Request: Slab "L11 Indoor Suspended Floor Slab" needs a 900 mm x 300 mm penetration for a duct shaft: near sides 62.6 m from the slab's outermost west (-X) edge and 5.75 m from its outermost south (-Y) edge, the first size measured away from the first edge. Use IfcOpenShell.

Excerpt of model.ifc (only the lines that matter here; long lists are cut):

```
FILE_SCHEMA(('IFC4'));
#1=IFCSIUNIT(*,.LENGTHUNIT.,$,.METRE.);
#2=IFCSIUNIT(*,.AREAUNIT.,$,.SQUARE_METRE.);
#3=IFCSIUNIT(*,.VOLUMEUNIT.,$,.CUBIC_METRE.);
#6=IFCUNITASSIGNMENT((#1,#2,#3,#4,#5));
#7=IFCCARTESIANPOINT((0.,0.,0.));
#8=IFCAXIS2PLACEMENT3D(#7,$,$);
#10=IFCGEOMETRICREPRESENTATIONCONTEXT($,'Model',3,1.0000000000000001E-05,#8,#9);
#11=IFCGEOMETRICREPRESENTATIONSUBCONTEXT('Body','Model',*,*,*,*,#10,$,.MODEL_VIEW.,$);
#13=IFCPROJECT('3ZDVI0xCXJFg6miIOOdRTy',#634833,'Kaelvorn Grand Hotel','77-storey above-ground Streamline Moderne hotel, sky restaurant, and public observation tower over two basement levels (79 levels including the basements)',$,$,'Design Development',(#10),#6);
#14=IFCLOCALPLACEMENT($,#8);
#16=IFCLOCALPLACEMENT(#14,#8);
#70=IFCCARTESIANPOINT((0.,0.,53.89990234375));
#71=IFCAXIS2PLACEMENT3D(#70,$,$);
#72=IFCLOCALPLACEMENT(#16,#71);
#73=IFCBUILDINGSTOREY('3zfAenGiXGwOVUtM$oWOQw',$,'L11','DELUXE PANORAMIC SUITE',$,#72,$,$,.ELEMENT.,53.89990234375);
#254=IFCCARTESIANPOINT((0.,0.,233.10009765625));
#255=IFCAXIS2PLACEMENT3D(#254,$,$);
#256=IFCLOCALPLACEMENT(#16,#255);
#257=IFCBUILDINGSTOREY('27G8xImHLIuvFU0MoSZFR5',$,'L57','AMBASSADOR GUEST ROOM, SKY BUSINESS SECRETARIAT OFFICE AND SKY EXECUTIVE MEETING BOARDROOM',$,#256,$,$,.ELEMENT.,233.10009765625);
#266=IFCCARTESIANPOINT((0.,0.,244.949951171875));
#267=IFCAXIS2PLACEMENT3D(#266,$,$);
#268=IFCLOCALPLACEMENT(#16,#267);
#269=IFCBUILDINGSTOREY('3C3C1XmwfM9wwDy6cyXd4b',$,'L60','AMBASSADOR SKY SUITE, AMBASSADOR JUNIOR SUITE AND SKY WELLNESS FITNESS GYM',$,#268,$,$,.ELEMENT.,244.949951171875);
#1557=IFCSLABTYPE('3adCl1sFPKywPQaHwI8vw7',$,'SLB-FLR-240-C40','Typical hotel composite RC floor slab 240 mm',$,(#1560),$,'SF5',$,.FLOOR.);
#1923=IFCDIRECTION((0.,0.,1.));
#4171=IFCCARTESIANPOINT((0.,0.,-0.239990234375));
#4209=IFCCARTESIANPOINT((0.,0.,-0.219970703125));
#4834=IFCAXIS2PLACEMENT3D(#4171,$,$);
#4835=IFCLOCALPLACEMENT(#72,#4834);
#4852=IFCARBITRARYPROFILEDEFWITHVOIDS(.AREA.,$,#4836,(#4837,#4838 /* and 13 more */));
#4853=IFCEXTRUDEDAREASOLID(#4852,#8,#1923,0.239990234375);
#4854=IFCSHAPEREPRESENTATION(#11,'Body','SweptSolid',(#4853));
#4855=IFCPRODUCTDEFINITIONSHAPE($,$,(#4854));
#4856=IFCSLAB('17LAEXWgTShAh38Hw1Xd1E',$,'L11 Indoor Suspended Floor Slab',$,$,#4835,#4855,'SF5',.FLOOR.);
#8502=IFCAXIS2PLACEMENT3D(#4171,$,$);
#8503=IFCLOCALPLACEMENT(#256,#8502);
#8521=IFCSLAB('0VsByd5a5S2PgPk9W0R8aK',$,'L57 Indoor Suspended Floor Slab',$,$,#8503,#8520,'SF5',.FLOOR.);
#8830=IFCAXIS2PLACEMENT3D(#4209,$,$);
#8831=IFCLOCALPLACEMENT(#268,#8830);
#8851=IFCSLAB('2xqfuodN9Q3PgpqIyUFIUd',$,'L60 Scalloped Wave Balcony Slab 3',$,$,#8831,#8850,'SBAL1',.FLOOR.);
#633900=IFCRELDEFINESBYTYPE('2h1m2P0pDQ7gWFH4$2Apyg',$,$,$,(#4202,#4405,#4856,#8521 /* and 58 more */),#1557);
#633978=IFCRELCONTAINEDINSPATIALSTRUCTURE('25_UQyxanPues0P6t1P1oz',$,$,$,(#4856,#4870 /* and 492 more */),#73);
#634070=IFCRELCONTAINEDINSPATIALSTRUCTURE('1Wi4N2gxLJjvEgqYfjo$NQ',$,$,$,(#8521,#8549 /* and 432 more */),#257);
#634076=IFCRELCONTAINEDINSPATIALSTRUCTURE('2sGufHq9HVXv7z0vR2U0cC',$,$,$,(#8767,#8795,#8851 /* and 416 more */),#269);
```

```python
import numpy as np
import ifcopenshell
import ifcopenshell.api.feature
import ifcopenshell.api.geometry
import ifcopenshell.api.root
import ifcopenshell.geom
import ifcopenshell.util.placement
import ifcopenshell.util.representation
import ifcopenshell.util.shape
import ifcopenshell.util.unit

model = ifcopenshell.open("model.ifc")
unit_scale = ifcopenshell.util.unit.calculate_unit_scale(model)
settings = ifcopenshell.geom.settings()


def volume(element):
    """Net volume in cubic metres, openings subtracted."""
    shape = ifcopenshell.geom.create_shape(settings, element)
    return ifcopenshell.util.shape.get_volume(shape.geometry)


slab = model.by_guid("17LAEXWgTShAh38Hw1Xd1E")
before = volume(slab)

# Extent in the slab's own axes, in metres. The edges named are its -X and -Y sides.
slab_shape = ifcopenshell.geom.create_shape(settings, slab)
vertices = ifcopenshell.util.shape.get_vertices(slab_shape.geometry)
x_min, y_min, bottom = vertices.min(axis=0)
top = vertices[:, 2].max()

opening = ifcopenshell.api.root.create_entity(model, ifc_class="IfcOpeningElement", name="Duct shaft opening", predefined_type="OPENING")
context = ifcopenshell.util.representation.get_context(model, "Model", "Body", "MODEL_VIEW")
width, depth = 0.9, 0.3
outline = [(0.0, 0.0), (width, 0.0), (width, depth), (0.0, depth), (0.0, 0.0)]
# Overshoot both faces by 50 mm so the cut is clean.
shape = ifcopenshell.api.geometry.add_slab_representation(
    model, context=context, depth=top - bottom + 0.1, polyline=outline
)
ifcopenshell.api.geometry.assign_representation(model, product=opening, representation=shape)

matrix = ifcopenshell.util.placement.get_local_placement(slab.ObjectPlacement)
matrix[:, 3] = matrix @ np.append(np.array([x_min + 62.6, y_min + 5.75, bottom - 0.05]) / unit_scale, 1.0)
ifcopenshell.api.geometry.edit_object_placement(model, product=opening, matrix=matrix, is_si=False)
ifcopenshell.api.feature.add_feature(model, feature=opening, element=slab)

after = volume(slab)

print(f"slab volume {before:.3f} -> {after:.3f} m3")

model.write("model_edited.ifc")
```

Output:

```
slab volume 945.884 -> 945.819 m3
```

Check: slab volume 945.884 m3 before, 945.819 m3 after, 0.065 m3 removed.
